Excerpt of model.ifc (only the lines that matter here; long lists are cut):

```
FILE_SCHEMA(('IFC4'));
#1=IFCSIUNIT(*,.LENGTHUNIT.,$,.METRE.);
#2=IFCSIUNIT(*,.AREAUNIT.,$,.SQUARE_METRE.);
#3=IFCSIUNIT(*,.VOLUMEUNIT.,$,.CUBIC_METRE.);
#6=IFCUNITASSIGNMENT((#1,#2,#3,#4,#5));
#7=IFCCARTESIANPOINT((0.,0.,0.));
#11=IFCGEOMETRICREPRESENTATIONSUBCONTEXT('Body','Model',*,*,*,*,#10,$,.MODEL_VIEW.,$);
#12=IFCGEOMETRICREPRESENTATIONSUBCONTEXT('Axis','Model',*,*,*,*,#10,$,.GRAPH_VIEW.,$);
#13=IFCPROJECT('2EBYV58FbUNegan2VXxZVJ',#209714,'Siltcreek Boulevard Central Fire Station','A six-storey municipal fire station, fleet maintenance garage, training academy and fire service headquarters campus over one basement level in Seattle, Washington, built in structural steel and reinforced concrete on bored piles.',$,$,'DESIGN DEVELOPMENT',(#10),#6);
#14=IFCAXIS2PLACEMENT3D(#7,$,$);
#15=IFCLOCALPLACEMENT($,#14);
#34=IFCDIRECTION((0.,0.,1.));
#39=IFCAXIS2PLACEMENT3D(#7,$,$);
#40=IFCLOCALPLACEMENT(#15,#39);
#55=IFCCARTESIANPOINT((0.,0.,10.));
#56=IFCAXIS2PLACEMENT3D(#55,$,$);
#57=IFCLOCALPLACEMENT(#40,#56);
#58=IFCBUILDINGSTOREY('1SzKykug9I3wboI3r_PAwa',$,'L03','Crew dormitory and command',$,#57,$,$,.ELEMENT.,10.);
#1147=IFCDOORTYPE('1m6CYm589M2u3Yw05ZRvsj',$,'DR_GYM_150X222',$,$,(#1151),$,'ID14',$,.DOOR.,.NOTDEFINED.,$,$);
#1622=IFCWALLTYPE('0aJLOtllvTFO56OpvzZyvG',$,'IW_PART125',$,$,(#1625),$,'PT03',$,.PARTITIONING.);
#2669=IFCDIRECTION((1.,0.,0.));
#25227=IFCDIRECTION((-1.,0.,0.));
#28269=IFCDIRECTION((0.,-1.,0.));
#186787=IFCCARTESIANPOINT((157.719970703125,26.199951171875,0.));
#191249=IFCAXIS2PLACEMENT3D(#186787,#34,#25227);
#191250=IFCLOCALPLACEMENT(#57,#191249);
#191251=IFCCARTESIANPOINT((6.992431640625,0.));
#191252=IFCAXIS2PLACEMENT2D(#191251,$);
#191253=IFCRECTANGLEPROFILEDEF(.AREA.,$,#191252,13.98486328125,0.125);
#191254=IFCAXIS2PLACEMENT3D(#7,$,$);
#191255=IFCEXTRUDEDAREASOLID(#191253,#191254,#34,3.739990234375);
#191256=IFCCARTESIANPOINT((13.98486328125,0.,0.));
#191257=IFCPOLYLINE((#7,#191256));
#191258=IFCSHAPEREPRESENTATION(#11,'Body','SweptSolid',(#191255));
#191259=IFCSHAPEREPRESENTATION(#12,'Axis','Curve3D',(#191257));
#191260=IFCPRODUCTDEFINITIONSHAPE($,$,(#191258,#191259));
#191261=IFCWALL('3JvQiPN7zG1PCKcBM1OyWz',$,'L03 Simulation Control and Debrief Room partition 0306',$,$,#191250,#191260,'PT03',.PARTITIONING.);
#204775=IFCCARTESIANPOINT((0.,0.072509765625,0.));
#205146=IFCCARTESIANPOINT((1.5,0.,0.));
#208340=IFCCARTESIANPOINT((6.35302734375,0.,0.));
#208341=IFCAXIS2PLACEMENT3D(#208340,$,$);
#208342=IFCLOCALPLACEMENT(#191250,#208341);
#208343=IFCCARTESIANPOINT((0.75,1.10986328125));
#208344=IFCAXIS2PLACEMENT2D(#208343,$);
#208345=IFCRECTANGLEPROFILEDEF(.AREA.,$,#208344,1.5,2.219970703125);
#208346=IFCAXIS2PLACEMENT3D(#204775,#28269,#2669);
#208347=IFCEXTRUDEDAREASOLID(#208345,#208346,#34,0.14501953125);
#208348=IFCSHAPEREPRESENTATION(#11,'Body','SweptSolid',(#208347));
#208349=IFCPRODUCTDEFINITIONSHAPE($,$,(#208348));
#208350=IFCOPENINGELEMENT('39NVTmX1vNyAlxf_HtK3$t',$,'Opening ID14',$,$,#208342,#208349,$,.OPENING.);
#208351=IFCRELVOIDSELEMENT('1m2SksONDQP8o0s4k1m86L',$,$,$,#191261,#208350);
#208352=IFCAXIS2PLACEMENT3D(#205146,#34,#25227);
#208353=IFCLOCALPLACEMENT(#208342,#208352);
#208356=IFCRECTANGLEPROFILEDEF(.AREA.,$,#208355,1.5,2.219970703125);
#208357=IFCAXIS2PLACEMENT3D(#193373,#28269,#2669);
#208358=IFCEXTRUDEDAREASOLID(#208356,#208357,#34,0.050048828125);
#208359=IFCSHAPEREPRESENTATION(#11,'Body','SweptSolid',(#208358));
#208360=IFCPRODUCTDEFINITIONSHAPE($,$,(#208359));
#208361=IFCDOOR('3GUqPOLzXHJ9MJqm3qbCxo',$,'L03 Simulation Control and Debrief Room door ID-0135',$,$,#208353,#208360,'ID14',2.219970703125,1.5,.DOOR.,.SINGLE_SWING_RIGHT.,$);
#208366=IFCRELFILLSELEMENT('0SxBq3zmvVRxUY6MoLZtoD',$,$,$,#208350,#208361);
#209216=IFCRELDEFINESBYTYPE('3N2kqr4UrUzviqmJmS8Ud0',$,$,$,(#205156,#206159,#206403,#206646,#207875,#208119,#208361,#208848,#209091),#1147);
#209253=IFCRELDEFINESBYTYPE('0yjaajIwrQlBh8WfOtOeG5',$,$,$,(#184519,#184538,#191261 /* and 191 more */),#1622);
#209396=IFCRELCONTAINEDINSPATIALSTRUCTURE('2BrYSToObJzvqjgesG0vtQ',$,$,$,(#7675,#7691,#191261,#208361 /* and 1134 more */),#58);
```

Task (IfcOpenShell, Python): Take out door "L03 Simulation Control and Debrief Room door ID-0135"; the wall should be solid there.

```python
import ifcopenshell
import ifcopenshell.api.feature
import ifcopenshell.api.root
import ifcopenshell.geom
import ifcopenshell.util.shape

model = ifcopenshell.open("model.ifc")
settings = ifcopenshell.geom.settings()


def volume(element):
    """Net volume in cubic metres, openings subtracted."""
    shape = ifcopenshell.geom.create_shape(settings, element)
    return ifcopenshell.util.shape.get_volume(shape.geometry)


door = model.by_guid("3GUqPOLzXHJ9MJqm3qbCxo")
opening = door.FillsVoids[0].RelatingOpeningElement
wall = opening.VoidsElements[0].RelatingBuildingElement
before = volume(wall)

ifcopenshell.api.root.remove_product(model, product=door)
ifcopenshell.api.feature.remove_feature(model, feature=opening)

after = volume(wall)

print(f"wall volume {before:.3f} -> {after:.3f} m3")

model.write("model_edited.ifc")
```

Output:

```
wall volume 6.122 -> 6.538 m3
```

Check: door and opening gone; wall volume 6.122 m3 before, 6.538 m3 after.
